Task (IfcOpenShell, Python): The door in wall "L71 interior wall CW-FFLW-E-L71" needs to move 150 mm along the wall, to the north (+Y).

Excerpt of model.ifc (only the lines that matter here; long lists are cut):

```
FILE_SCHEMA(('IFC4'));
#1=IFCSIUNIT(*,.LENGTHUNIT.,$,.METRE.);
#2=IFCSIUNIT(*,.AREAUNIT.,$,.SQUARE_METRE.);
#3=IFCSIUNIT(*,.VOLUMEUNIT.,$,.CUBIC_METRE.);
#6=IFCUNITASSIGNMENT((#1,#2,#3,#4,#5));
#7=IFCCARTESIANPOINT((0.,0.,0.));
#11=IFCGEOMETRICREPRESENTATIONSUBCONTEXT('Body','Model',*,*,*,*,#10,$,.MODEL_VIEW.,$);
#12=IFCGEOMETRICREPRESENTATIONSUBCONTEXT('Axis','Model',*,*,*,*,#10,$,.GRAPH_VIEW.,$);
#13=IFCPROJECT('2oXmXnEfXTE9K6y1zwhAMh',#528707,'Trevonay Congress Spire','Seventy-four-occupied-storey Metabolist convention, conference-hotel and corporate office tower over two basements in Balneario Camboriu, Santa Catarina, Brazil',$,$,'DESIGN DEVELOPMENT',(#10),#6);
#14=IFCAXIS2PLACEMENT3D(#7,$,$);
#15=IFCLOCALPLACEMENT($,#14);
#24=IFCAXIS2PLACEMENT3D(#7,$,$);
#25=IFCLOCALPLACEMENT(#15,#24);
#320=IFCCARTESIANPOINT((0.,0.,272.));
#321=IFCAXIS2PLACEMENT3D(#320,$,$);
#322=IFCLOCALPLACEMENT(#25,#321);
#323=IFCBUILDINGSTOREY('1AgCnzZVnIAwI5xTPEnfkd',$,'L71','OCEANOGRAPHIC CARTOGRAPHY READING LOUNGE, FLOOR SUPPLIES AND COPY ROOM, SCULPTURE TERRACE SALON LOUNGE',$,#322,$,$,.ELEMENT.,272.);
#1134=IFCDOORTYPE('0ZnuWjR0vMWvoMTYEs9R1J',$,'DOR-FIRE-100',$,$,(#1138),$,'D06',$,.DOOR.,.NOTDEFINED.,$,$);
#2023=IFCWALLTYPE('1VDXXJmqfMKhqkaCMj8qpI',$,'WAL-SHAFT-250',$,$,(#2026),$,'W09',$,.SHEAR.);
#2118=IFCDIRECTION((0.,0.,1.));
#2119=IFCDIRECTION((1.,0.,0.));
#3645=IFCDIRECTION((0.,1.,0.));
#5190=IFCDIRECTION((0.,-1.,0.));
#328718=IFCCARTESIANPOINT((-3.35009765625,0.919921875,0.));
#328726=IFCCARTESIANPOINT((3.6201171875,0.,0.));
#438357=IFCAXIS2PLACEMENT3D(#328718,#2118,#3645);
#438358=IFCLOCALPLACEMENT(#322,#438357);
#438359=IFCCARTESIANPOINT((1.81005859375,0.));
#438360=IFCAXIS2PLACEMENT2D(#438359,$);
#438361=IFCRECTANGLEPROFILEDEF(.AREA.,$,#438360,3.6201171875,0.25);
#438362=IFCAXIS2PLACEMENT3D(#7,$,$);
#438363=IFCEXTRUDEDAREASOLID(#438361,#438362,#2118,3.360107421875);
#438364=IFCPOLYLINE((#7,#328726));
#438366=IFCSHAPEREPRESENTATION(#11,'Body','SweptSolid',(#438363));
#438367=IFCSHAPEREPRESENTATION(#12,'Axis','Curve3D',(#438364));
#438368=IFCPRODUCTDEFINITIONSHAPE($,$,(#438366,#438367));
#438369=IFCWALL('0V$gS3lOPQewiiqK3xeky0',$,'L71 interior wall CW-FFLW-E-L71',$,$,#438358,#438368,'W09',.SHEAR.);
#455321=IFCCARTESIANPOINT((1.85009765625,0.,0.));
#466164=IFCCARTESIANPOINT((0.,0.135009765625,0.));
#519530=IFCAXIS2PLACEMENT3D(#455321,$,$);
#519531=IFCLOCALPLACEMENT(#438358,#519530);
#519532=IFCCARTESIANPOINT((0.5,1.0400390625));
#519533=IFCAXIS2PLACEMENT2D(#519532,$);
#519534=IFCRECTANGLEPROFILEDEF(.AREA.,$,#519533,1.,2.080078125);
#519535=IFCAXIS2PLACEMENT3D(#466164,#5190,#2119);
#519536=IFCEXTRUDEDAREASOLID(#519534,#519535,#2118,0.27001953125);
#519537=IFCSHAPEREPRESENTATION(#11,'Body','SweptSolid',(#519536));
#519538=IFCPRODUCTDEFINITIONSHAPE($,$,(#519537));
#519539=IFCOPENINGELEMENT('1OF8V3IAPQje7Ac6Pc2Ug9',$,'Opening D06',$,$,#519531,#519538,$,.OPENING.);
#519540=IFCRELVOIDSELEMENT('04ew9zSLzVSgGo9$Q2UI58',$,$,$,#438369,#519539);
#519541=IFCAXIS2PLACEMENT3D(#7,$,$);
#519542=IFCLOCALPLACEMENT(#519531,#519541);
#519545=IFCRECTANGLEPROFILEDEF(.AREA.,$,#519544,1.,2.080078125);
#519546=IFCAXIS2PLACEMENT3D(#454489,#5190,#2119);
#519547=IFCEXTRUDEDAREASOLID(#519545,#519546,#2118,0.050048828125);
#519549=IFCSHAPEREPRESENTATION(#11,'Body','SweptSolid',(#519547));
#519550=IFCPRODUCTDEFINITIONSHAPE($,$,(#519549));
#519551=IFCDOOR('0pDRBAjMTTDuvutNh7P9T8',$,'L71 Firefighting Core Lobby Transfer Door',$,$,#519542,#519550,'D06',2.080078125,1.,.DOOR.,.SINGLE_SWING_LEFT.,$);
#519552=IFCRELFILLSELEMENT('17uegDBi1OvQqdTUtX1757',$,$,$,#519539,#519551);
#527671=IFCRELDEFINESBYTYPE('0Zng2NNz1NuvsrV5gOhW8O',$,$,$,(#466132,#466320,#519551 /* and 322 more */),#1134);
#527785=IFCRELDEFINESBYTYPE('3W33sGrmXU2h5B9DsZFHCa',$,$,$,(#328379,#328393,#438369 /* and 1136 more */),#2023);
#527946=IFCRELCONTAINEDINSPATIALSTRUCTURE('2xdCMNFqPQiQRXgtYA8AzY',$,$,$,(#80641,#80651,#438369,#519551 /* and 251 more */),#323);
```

```python
import ifcopenshell
import ifcopenshell.api.geometry
import ifcopenshell.util.placement
import ifcopenshell.util.unit

model = ifcopenshell.open("model.ifc")
unit_scale = ifcopenshell.util.unit.calculate_unit_scale(model)

door = model.by_guid("0pDRBAjMTTDuvutNh7P9T8")
opening = door.FillsVoids[0].RelatingOpeningElement
wall = opening.VoidsElements[0].RelatingBuildingElement

wall_matrix = ifcopenshell.util.placement.get_local_placement(wall.ObjectPlacement)
shift = wall_matrix[:3, 0] * 0.15 / unit_scale
before = ifcopenshell.util.placement.get_local_placement(door.ObjectPlacement)[:3, 3].copy()

# The door is placed relative to its opening, so it follows when the opening moves.
matrix = ifcopenshell.util.placement.get_local_placement(opening.ObjectPlacement)
matrix[:3, 3] += shift
ifcopenshell.api.geometry.edit_object_placement(
    model, product=opening, matrix=matrix, is_si=False, should_transform_children=True
)

after = ifcopenshell.util.placement.get_local_placement(door.ObjectPlacement)[:3, 3]
print("door moved by", (after - before).round(3) + 0.0)

model.write("model-out.ifc")
```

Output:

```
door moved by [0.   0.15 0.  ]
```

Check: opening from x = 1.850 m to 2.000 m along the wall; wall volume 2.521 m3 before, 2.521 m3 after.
